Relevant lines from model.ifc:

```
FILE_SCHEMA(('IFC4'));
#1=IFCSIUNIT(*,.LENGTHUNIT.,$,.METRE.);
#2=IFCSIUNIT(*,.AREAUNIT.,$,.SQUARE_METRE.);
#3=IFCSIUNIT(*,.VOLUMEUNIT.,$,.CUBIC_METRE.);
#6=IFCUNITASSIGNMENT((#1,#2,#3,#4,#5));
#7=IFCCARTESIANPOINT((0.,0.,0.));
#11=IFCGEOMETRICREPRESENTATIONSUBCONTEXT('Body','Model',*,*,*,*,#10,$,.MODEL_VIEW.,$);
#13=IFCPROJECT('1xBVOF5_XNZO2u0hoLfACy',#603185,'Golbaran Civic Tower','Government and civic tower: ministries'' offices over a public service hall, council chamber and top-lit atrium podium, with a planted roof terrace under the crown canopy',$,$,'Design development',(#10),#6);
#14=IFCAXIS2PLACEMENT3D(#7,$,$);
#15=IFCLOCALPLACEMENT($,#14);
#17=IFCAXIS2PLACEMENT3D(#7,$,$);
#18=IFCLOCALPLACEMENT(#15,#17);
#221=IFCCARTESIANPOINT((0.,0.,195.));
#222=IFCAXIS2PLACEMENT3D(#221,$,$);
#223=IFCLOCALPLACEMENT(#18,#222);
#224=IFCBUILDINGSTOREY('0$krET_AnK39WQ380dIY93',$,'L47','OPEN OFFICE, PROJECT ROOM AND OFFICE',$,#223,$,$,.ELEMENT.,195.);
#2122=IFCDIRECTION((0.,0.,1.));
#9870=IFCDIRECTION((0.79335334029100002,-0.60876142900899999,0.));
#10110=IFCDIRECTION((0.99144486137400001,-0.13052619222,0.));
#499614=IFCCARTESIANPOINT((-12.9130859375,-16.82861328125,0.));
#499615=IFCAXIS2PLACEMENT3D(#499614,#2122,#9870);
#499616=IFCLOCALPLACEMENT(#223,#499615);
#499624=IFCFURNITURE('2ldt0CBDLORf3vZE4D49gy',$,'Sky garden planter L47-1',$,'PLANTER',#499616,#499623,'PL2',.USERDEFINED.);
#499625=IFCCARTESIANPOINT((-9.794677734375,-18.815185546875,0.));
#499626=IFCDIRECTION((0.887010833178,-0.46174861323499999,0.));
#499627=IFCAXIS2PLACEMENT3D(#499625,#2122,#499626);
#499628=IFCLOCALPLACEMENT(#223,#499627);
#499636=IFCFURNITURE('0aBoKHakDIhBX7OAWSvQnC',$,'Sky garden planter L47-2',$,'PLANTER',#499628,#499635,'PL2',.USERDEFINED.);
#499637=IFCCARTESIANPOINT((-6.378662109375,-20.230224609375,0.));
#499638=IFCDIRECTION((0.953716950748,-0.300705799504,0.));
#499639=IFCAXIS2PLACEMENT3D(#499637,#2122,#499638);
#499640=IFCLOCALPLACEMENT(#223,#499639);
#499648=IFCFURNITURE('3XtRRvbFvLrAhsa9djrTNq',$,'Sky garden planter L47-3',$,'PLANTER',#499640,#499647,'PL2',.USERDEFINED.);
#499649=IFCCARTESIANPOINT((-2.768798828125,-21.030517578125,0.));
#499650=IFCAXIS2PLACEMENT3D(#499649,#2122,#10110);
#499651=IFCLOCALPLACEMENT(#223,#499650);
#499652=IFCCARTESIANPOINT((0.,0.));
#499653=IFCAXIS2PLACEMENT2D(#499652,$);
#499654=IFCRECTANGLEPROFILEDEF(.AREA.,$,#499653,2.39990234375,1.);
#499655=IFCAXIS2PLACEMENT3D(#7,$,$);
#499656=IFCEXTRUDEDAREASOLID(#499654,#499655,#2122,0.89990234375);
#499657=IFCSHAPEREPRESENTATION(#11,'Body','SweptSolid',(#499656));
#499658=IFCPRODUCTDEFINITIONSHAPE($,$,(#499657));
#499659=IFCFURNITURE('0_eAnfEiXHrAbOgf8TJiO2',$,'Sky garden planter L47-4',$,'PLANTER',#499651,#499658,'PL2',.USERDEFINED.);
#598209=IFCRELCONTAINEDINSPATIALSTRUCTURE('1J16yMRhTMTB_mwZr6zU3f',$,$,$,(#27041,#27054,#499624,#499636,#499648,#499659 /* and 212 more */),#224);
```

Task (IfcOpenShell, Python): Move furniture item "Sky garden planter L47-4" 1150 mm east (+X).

```python
import ifcopenshell
import ifcopenshell.api.geometry
import ifcopenshell.util.placement

model = ifcopenshell.open("model.ifc")

item = model.by_guid("0_eAnfEiXHrAbOgf8TJiO2")
matrix = ifcopenshell.util.placement.get_local_placement(item.ObjectPlacement)
matrix[0, 3] += 1.15
ifcopenshell.api.geometry.edit_object_placement(model, product=item, matrix=matrix, is_si=False)

print(ifcopenshell.util.placement.get_local_placement(item.ObjectPlacement).round(3) + 0.0)

model.write("model_edited.ifc")
```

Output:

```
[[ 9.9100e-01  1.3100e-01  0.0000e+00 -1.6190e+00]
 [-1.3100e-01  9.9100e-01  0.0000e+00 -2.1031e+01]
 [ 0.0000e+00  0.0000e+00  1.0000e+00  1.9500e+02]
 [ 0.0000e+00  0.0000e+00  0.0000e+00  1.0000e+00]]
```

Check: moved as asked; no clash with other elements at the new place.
